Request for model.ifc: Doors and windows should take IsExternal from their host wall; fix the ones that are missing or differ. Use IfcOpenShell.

First a look at what the model holds.

```python
import ifcopenshell
import ifcopenshell.util.element

model = ifcopenshell.open("model.ifc")
print(model.schema)
seen = {}
for e in model.by_type("IfcDoor") + model.by_type("IfcWindow"):
    if not e.FillsVoids:
        continue
    host = e.FillsVoids[0].RelatingOpeningElement.VoidsElements[0].RelatingBuildingElement
    own = ifcopenshell.util.element.get_pset(e, f"Pset_{e.is_a()[3:].removesuffix('StandardCase')}Common", "IsExternal")
    wall = ifcopenshell.util.element.get_pset(host, "Pset_WallCommon", "IsExternal")
    seen[e.is_a(), own, wall] = seen.get((e.is_a(), own, wall), 0) + 1
for (cls, own, wall), count in sorted(seen.items(), key=str):
    print(count, cls, "IsExternal:", own, "| host wall:", wall)
```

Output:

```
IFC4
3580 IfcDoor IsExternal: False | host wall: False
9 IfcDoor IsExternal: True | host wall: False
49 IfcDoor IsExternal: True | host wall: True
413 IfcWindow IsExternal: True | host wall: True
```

```python
import ifcopenshell
import ifcopenshell.api.pset
import ifcopenshell.util.element

model = ifcopenshell.open("model.ifc")

count = 0
for ifc_class, pset_name in (("IfcDoor", "Pset_DoorCommon"), ("IfcWindow", "Pset_WindowCommon")):
    for e in model.by_type(ifc_class):
        if not e.FillsVoids:
            continue
        host = e.FillsVoids[0].RelatingOpeningElement.VoidsElements[0].RelatingBuildingElement
        external = ifcopenshell.util.element.get_pset(host, "Pset_WallCommon", "IsExternal")
        if external is None or ifcopenshell.util.element.get_pset(e, pset_name, "IsExternal") == external:
            continue
        pset = ifcopenshell.api.pset.add_pset(model, product=e, name=pset_name)
        ifcopenshell.api.pset.edit_pset(model, pset=pset, properties={"IsExternal": external})
        count += 1

print(count, "updated")

model.write("model_edited.ifc")
```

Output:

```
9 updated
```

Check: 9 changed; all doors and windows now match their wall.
